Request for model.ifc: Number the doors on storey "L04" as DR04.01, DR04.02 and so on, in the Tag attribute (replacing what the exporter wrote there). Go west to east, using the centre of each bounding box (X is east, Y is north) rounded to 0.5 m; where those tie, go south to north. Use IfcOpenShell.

First a look at what the model holds.

```python
import ifcopenshell
import ifcopenshell.util.element
import ifcopenshell.util.placement

model = ifcopenshell.open("model.ifc")
print(model.schema)
storey = next(s for s in model.by_type("IfcBuildingStorey") if s.Name == "L04")
doors = [e for e in ifcopenshell.util.element.get_decomposition(storey) if e.is_a("IfcDoor")]
for e in sorted(doors, key=lambda e: e.id()):
    origin = ifcopenshell.util.placement.get_local_placement(e.ObjectPlacement)[:3, 3]
    print(e.id(), e.Tag, e.Name, origin.round(2) + 0.0, sep=" | ")
```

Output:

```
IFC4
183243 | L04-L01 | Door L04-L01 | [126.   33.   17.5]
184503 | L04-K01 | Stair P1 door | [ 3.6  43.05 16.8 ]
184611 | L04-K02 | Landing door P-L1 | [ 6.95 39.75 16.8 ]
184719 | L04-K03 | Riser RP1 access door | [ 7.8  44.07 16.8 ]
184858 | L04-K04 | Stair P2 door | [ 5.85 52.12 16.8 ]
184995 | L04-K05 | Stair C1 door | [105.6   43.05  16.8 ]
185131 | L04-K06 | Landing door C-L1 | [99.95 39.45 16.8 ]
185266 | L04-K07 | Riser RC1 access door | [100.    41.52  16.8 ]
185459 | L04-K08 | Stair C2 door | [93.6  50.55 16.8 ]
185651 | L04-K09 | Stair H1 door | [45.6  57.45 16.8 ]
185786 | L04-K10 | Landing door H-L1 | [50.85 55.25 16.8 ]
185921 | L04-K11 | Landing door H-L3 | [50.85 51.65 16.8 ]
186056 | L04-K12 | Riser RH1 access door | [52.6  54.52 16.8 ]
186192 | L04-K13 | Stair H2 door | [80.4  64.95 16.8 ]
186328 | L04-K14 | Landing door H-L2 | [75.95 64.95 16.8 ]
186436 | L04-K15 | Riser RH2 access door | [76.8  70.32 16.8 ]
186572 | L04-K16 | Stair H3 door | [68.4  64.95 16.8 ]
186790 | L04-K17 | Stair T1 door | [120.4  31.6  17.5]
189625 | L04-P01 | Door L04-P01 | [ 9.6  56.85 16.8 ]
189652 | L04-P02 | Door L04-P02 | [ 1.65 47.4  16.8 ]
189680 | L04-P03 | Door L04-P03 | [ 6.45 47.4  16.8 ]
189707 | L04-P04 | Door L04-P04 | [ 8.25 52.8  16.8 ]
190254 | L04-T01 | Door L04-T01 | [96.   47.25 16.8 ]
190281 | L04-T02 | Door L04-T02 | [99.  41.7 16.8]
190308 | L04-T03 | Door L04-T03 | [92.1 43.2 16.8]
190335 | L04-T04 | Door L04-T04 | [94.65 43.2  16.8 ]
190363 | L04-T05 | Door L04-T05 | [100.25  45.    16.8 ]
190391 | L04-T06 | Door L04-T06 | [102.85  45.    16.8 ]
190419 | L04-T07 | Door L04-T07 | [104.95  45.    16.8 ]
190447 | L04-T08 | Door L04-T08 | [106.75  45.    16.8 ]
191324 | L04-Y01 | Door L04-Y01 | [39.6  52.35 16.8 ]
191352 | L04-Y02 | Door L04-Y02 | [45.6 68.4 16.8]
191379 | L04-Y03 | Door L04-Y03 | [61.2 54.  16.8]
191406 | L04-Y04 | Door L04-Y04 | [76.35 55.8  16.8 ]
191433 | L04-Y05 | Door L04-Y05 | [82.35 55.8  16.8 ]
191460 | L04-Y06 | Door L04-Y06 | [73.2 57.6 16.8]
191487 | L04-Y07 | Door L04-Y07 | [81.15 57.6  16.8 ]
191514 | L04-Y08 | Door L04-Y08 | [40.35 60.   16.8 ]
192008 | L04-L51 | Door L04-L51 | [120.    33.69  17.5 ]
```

```python
import ifcopenshell
import ifcopenshell.geom
import ifcopenshell.util.element
import ifcopenshell.util.shape

model = ifcopenshell.open("model.ifc")
settings = ifcopenshell.geom.settings()
settings.set("use-world-coords", True)


def centre(element):
    shape = ifcopenshell.geom.create_shape(settings, element)
    return ifcopenshell.util.shape.get_bbox_centroid(shape.geometry)


storey = next(s for s in model.by_type("IfcBuildingStorey") if s.Name == "L04")
doors = [e for e in ifcopenshell.util.element.get_decomposition(storey) if e.is_a("IfcDoor")]

# Insertion points can sit at a corner or the storey origin, so sort by the geometry (in metres).
centres = {e: centre(e) for e in doors}
doors.sort(key=lambda e: (round(centres[e][0] / 0.5), centres[e][1]))

for i, e in enumerate(doors, start=1):
    number = f"DR04.{i:02d}"
    e.Tag = number
    print(e.id(), number)

model.write("model_rev.ifc")
```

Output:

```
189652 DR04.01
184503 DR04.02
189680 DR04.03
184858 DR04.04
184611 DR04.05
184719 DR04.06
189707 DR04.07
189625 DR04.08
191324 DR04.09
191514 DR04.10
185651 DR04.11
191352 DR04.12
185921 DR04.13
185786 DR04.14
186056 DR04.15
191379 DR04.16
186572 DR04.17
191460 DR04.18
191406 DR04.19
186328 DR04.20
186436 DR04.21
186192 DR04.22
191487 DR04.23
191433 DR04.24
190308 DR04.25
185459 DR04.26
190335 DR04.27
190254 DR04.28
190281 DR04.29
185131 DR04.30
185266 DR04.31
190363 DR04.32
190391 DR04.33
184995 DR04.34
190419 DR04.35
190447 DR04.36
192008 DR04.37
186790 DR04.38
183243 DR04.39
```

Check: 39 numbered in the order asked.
